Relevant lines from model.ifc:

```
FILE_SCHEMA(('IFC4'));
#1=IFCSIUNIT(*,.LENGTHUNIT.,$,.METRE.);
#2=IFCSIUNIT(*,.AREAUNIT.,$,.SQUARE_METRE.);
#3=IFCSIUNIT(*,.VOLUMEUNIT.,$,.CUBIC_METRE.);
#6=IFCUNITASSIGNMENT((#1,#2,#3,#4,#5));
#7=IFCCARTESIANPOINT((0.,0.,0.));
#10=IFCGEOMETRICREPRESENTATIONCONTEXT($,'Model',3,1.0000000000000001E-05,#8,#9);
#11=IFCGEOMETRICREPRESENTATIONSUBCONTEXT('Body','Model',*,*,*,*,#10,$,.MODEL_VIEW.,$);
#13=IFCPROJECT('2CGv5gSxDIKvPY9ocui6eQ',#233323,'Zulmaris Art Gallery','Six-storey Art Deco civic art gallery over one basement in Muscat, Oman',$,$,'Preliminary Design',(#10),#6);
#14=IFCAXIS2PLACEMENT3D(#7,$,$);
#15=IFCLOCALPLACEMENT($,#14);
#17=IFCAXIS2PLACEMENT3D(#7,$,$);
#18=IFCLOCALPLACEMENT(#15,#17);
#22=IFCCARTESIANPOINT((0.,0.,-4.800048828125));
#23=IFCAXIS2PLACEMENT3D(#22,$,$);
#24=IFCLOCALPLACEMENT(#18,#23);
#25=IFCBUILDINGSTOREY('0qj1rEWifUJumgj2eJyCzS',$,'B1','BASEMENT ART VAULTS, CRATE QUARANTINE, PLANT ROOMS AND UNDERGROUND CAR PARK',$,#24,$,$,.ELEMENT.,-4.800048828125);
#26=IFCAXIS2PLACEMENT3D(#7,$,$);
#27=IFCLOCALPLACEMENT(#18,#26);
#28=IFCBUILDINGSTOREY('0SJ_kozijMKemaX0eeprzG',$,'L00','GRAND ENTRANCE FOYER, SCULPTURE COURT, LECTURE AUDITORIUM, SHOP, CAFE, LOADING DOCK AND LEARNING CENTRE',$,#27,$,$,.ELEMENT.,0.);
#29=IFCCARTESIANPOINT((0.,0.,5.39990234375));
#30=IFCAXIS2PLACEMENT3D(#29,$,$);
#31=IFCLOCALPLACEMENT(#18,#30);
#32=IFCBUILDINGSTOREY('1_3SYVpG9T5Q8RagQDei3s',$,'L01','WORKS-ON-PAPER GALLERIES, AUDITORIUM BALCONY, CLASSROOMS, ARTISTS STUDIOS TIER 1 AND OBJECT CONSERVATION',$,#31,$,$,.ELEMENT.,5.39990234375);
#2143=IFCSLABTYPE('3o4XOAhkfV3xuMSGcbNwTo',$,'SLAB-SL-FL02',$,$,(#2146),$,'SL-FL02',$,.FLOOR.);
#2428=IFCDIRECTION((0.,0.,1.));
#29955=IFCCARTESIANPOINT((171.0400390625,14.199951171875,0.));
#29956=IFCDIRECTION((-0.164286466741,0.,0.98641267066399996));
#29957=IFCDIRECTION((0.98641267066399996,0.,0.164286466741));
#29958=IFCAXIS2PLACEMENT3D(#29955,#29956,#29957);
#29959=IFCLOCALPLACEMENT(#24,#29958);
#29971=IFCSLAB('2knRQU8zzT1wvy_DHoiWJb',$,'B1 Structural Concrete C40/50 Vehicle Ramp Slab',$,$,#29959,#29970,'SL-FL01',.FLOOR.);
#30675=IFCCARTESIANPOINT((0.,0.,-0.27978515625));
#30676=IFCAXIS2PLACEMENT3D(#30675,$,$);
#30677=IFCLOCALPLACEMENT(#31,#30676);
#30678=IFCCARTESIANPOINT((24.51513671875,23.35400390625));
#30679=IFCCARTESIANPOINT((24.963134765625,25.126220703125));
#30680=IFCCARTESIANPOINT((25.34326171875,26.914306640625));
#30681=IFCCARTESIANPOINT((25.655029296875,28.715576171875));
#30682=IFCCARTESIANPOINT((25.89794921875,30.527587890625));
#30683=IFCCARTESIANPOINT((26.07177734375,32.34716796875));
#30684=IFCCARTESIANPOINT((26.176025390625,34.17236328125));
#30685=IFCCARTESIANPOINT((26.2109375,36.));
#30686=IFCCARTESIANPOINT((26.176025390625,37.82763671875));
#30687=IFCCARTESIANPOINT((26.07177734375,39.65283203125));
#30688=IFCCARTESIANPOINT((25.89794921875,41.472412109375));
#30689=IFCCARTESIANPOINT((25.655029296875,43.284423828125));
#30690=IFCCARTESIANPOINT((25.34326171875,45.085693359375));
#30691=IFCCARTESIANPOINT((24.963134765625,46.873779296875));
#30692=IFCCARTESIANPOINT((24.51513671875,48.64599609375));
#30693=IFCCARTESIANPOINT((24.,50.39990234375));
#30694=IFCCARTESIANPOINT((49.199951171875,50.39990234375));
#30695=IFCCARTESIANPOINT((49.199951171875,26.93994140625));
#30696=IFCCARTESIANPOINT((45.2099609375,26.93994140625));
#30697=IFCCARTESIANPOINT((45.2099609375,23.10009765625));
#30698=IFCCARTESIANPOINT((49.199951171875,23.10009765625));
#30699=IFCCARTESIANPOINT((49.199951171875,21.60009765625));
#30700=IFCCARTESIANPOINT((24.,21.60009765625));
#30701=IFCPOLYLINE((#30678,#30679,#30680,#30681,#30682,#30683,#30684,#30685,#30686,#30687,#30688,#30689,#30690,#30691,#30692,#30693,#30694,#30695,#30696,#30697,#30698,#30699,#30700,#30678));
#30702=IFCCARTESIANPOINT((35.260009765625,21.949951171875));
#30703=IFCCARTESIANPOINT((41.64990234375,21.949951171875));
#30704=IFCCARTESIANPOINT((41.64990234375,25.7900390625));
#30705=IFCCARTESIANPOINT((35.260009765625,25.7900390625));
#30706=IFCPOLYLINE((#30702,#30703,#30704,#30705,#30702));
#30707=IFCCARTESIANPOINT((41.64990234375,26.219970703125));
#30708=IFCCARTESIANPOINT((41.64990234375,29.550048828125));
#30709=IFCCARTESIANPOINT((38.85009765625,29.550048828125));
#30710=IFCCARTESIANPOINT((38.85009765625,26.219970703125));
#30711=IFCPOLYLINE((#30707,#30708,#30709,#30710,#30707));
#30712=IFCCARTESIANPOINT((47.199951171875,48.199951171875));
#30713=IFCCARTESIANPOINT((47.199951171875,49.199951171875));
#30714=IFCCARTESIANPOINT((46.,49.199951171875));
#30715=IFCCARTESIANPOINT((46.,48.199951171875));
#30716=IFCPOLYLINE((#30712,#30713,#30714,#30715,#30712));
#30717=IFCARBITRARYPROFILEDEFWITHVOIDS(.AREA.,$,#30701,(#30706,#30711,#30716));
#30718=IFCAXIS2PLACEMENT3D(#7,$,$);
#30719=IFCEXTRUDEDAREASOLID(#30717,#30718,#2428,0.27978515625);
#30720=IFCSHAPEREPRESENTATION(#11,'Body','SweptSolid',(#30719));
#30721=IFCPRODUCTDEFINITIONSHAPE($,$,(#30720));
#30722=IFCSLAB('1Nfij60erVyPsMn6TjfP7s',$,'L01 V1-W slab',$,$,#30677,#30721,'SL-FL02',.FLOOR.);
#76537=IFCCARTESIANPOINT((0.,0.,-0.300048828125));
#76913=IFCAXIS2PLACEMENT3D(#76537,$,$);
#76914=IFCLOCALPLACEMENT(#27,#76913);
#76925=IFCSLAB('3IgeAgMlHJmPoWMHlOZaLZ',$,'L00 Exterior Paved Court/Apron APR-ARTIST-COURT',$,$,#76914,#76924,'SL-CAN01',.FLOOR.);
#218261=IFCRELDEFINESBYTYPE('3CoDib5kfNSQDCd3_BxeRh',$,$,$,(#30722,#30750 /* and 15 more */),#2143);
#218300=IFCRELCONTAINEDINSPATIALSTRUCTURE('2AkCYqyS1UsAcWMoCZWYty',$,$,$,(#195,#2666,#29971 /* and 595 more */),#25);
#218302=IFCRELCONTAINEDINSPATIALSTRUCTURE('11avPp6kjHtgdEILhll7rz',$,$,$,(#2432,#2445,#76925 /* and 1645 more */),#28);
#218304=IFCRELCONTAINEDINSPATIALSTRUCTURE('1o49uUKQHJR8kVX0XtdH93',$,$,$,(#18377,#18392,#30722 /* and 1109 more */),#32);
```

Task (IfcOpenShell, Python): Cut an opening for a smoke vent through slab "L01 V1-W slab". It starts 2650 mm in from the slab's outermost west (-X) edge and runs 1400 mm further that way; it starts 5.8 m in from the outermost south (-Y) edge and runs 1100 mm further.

```python
import numpy as np
import ifcopenshell
import ifcopenshell.api.feature
import ifcopenshell.api.geometry
import ifcopenshell.api.root
import ifcopenshell.geom
import ifcopenshell.util.placement
import ifcopenshell.util.representation
import ifcopenshell.util.shape
import ifcopenshell.util.unit

model = ifcopenshell.open("model.ifc")
unit_scale = ifcopenshell.util.unit.calculate_unit_scale(model)
settings = ifcopenshell.geom.settings()


def volume(element):
    """Net volume in cubic metres, openings subtracted."""
    shape = ifcopenshell.geom.create_shape(settings, element)
    return ifcopenshell.util.shape.get_volume(shape.geometry)


slab = model.by_guid("1Nfij60erVyPsMn6TjfP7s")
before = volume(slab)

# Extent in the slab's own axes, in metres. The edges named are its -X and -Y sides.
slab_shape = ifcopenshell.geom.create_shape(settings, slab)
vertices = ifcopenshell.util.shape.get_vertices(slab_shape.geometry)
x_min, y_min, bottom = vertices.min(axis=0)
top = vertices[:, 2].max()

opening = ifcopenshell.api.root.create_entity(model, ifc_class="IfcOpeningElement", name="Smoke vent opening", predefined_type="OPENING")
context = ifcopenshell.util.representation.get_context(model, "Model", "Body", "MODEL_VIEW")
width, depth = 1.4, 1.1
outline = [(0.0, 0.0), (width, 0.0), (width, depth), (0.0, depth), (0.0, 0.0)]
# Overshoot both faces by 50 mm so the cut is clean.
shape = ifcopenshell.api.geometry.add_slab_representation(
    model, context=context, depth=top - bottom + 0.1, polyline=outline
)
ifcopenshell.api.geometry.assign_representation(model, product=opening, representation=shape)

matrix = ifcopenshell.util.placement.get_local_placement(slab.ObjectPlacement)
matrix[:, 3] = matrix @ np.append(np.array([x_min + 2.65, y_min + 5.8, bottom - 0.05]) / unit_scale, 1.0)
ifcopenshell.api.geometry.edit_object_placement(model, product=opening, matrix=matrix, is_si=False)
ifcopenshell.api.feature.add_feature(model, feature=opening, element=slab)

after = volume(slab)

print(f"slab volume {before:.3f} -> {after:.3f} m3")

model.write("model-out.ifc")
```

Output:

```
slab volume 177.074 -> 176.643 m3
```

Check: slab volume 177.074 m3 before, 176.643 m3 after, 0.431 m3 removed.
